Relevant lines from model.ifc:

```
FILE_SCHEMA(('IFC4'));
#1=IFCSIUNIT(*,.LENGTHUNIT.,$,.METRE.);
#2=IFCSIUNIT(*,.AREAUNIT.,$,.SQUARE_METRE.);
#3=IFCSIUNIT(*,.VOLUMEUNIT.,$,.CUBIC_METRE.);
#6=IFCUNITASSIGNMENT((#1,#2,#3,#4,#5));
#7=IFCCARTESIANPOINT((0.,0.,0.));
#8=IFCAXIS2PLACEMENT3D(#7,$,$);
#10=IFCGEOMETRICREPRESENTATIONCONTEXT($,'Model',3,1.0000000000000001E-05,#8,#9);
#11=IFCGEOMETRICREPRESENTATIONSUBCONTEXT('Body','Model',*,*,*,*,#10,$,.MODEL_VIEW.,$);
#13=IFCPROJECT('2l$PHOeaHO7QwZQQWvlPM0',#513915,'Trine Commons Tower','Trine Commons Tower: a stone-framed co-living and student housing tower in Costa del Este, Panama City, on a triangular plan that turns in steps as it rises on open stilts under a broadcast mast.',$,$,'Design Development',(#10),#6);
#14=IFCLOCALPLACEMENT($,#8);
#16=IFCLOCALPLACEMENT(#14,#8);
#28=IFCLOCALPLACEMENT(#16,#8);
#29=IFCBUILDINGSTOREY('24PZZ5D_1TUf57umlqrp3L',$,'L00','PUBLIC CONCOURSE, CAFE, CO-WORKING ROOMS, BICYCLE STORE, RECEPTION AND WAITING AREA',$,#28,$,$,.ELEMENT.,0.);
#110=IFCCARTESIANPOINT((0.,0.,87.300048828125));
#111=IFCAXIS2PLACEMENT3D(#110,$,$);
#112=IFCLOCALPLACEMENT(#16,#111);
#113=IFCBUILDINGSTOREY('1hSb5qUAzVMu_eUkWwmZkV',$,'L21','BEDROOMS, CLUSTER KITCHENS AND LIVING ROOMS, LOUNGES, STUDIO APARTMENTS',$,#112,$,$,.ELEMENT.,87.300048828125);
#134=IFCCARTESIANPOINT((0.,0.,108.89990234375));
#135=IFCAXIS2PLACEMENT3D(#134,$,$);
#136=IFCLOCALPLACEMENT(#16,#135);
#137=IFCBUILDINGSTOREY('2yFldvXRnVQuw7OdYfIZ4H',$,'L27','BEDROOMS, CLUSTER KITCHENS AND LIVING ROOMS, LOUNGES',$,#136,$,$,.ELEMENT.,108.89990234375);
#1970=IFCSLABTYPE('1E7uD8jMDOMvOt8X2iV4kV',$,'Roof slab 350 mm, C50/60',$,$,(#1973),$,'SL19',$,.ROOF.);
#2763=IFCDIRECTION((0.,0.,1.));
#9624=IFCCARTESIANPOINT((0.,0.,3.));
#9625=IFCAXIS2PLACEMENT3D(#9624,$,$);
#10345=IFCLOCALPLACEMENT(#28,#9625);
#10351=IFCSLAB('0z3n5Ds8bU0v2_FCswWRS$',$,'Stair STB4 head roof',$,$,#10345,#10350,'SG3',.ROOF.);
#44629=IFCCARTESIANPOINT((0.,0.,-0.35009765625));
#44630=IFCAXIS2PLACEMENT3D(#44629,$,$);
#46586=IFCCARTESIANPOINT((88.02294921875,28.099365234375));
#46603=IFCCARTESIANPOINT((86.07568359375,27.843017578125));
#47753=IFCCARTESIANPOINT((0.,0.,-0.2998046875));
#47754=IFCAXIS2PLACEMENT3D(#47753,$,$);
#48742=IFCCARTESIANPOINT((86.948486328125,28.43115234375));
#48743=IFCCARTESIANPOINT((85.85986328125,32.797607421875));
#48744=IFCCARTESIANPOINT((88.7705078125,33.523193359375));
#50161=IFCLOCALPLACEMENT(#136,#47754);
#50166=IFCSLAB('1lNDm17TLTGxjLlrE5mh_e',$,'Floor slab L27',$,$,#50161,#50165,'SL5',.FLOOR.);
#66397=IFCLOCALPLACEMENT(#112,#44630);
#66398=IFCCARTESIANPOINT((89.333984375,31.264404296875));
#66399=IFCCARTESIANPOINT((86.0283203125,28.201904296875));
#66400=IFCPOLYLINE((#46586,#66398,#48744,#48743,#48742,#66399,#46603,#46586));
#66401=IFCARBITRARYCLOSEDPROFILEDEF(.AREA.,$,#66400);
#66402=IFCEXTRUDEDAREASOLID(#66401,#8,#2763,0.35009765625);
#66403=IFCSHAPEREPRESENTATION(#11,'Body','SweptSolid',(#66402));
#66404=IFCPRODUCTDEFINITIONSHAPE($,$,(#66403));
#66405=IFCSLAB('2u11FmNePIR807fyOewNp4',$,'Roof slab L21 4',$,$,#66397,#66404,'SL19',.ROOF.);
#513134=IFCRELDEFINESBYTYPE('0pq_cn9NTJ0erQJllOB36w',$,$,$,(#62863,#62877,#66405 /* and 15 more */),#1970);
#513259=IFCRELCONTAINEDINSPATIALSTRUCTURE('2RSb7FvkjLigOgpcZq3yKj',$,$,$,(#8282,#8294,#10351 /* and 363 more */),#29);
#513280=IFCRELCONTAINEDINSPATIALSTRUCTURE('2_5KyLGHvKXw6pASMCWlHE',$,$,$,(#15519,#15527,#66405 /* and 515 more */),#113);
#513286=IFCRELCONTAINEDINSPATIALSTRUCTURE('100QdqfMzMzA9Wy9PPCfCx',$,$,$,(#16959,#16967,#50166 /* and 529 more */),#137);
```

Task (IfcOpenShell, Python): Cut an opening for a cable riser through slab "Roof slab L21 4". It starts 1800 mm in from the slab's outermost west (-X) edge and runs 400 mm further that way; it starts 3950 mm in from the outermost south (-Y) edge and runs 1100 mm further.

```python
import numpy as np
import ifcopenshell
import ifcopenshell.api.feature
import ifcopenshell.api.geometry
import ifcopenshell.api.root
import ifcopenshell.geom
import ifcopenshell.util.placement
import ifcopenshell.util.representation
import ifcopenshell.util.shape
import ifcopenshell.util.unit

model = ifcopenshell.open("model.ifc")
unit_scale = ifcopenshell.util.unit.calculate_unit_scale(model)
settings = ifcopenshell.geom.settings()


def volume(element):
    """Net volume in cubic metres, openings subtracted."""
    shape = ifcopenshell.geom.create_shape(settings, element)
    return ifcopenshell.util.shape.get_volume(shape.geometry)


slab = model.by_id(66405)
before = volume(slab)

# Extent in the slab's own axes, in metres. The edges named are its -X and -Y sides.
slab_shape = ifcopenshell.geom.create_shape(settings, slab)
vertices = ifcopenshell.util.shape.get_vertices(slab_shape.geometry)
x_min, y_min, bottom = vertices.min(axis=0)
top = vertices[:, 2].max()

opening = ifcopenshell.api.root.create_entity(model, ifc_class="IfcOpeningElement", name="Cable riser opening", predefined_type="OPENING")
context = ifcopenshell.util.representation.get_context(model, "Model", "Body", "MODEL_VIEW")
width, depth = 0.4, 1.1
outline = [(0.0, 0.0), (width, 0.0), (width, depth), (0.0, depth), (0.0, 0.0)]
# Overshoot both faces by 50 mm so the cut is clean.
shape = ifcopenshell.api.geometry.add_slab_representation(
    model, context=context, depth=top - bottom + 0.1, polyline=outline
)
ifcopenshell.api.geometry.assign_representation(model, product=opening, representation=shape)

matrix = ifcopenshell.util.placement.get_local_placement(slab.ObjectPlacement)
matrix[:, 3] = matrix @ np.append(np.array([x_min + 1.8, y_min + 3.95, bottom - 0.05]) / unit_scale, 1.0)
ifcopenshell.api.geometry.edit_object_placement(model, product=opening, matrix=matrix, is_si=False)
ifcopenshell.api.feature.add_feature(model, feature=opening, element=slab)

after = volume(slab)

print(f"slab volume {before:.3f} -> {after:.3f} m3")

model.write("model-out.ifc")
```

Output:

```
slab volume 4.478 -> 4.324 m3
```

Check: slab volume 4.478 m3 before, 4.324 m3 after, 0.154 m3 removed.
